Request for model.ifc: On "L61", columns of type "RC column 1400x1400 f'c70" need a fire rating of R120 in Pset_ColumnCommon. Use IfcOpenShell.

First a look at what the model holds.

```python
import ifcopenshell
import ifcopenshell.util.element

model = ifcopenshell.open("model.ifc")
print(model.schema)
storey = next(s for s in model.by_type("IfcBuildingStorey") if s.Name == "L61")
columns = [e for e in ifcopenshell.util.element.get_decomposition(storey) if e.is_a("IfcColumn")]
seen = {}
for e in columns:
    element_type = ifcopenshell.util.element.get_type(e)
    key = (element_type.Name if element_type != e and element_type else None, ifcopenshell.util.element.get_pset(e, "Pset_ColumnCommon", "FireRating"))
    seen[key] = seen.get(key, 0) + 1
for (name, value), count in sorted(seen.items(), key=str):
    print(count, "x", name, "|", value)
```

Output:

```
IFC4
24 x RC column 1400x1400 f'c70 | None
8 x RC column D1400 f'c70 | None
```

```python
import ifcopenshell
import ifcopenshell.api.pset
import ifcopenshell.util.element

model = ifcopenshell.open("model.ifc")

storey = next(s for s in model.by_type("IfcBuildingStorey") if s.Name == "L61")
columns = [e for e in ifcopenshell.util.element.get_decomposition(storey) if e.is_a("IfcColumn")]

count = 0
for e in columns:
    element_type = ifcopenshell.util.element.get_type(e)
    if element_type in (None, e) or element_type.Name != "RC column 1400x1400 f'c70":
        continue
    found = ifcopenshell.util.element.get_pset(e, "Pset_ColumnCommon", should_inherit=False)
    if found:
        pset = model.by_id(found["id"])
        if len(ifcopenshell.util.element.get_elements_by_pset(pset)) > 1:
            pset = ifcopenshell.api.pset.unshare_pset(model, products=[e], pset=pset)[0]
    else:
        pset = ifcopenshell.api.pset.add_pset(model, product=e, name="Pset_ColumnCommon")
    ifcopenshell.api.pset.edit_pset(model, pset=pset, properties={"FireRating": "R120"})
    count += 1

print(count, "columns updated")

model.write("model_updated.ifc")
```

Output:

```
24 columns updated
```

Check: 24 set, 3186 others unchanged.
